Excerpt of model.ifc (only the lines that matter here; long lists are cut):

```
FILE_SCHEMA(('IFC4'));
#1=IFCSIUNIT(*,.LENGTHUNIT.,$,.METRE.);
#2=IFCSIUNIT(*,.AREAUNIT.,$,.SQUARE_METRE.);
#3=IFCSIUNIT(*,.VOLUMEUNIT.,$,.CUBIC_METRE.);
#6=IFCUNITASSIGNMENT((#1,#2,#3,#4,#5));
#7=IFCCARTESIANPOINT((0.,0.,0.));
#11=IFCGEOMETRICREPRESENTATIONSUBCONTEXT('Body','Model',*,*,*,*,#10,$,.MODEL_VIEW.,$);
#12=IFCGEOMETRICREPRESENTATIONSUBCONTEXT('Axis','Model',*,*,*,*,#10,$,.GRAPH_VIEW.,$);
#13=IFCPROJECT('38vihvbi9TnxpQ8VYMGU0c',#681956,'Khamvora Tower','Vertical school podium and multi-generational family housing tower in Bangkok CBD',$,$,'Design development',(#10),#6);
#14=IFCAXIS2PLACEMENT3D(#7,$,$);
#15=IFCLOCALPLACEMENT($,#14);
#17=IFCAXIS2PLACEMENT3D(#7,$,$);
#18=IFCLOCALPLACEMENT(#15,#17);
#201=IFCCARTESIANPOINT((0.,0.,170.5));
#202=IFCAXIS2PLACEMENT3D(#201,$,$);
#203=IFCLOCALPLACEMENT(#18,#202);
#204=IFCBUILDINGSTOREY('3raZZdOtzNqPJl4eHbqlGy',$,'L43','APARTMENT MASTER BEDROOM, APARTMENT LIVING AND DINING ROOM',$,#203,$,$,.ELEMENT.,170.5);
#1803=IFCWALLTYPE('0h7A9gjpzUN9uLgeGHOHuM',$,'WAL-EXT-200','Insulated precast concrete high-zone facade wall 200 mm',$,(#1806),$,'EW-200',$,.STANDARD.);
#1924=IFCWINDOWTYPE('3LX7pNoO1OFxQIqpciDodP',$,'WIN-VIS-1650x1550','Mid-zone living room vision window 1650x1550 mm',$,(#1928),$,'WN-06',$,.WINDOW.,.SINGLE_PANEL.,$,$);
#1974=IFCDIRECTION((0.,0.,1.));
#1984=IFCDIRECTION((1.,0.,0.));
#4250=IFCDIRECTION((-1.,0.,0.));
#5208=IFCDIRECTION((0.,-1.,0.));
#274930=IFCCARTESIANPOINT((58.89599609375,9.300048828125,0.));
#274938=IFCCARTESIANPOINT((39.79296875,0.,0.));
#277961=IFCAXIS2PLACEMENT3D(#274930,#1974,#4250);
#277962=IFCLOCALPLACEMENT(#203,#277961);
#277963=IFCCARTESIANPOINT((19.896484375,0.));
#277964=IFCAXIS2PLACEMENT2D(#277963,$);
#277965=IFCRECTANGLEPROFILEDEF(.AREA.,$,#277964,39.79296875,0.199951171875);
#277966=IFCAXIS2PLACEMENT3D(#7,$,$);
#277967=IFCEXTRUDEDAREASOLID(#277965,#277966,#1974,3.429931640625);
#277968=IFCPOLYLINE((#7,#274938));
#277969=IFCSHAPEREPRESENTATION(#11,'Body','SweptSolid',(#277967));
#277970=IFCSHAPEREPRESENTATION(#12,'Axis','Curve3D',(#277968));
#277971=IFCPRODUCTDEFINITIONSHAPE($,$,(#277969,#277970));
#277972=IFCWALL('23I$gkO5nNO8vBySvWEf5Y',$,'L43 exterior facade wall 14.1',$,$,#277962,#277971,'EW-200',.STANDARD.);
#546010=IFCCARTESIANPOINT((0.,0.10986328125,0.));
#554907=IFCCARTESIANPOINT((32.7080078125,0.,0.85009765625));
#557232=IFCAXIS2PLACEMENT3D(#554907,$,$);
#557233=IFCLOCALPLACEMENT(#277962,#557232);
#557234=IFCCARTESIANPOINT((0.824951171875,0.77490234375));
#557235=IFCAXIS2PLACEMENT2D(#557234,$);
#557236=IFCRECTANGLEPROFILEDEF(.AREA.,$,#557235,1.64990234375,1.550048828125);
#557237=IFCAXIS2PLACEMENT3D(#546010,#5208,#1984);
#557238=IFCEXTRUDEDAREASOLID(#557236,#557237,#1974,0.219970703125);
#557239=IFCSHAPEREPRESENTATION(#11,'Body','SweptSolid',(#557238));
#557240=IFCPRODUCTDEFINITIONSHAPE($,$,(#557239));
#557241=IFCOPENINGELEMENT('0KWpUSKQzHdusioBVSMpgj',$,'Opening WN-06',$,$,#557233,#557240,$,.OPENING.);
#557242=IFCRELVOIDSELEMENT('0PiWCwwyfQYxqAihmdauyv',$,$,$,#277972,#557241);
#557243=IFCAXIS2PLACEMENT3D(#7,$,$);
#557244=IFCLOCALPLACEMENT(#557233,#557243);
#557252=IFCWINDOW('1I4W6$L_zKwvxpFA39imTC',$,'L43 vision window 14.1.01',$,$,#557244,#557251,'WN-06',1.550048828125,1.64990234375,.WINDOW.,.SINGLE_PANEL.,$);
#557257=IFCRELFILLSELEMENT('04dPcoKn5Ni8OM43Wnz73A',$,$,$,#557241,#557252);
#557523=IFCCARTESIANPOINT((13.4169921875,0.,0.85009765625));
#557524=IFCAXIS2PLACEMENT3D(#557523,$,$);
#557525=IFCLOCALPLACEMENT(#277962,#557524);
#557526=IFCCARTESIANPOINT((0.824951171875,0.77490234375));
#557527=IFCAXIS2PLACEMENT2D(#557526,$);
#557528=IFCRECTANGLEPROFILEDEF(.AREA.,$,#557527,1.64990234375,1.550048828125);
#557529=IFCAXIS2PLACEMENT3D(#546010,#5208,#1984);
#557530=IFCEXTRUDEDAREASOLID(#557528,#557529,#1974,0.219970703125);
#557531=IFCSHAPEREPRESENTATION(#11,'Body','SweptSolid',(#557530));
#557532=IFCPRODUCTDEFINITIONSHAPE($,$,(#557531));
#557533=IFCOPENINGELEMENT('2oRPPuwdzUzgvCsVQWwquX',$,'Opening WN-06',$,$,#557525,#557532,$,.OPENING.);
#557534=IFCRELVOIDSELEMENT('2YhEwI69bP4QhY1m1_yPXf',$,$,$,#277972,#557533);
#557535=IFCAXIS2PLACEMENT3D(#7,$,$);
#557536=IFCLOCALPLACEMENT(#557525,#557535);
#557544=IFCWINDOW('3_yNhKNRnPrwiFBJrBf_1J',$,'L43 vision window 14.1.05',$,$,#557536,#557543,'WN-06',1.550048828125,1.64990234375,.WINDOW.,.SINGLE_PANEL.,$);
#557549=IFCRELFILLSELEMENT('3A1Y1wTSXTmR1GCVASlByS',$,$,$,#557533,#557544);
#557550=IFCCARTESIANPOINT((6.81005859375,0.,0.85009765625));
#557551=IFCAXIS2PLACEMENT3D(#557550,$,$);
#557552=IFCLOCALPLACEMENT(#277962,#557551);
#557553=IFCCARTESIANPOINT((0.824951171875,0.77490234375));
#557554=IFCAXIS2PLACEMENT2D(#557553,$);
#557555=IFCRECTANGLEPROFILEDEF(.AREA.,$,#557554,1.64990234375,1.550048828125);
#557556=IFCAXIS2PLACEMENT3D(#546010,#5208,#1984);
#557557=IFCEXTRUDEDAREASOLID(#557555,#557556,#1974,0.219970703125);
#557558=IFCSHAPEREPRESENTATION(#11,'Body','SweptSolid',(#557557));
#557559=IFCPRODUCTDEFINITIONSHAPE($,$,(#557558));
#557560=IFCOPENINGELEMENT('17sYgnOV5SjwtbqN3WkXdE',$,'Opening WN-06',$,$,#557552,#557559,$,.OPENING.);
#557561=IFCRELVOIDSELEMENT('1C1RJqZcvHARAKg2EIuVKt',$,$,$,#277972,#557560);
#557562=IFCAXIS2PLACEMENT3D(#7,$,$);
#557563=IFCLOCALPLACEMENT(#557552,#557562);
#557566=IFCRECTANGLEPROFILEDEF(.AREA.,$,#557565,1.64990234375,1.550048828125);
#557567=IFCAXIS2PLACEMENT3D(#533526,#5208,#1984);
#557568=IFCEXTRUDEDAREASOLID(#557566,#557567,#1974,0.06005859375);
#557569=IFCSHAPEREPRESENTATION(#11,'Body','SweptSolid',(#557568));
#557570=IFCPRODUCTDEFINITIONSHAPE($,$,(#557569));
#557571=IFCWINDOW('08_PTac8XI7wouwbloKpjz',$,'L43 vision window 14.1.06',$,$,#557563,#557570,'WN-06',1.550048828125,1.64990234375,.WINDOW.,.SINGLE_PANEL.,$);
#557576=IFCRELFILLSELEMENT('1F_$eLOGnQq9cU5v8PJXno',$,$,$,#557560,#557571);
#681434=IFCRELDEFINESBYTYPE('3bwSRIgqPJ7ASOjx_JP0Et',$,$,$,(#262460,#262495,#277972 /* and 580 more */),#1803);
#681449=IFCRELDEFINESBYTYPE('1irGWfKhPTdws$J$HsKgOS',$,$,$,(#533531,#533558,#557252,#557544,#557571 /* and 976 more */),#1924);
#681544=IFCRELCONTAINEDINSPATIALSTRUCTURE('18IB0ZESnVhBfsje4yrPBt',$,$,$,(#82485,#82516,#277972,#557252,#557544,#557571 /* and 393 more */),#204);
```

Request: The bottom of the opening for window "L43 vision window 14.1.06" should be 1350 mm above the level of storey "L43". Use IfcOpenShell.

```python
import numpy as np
import ifcopenshell
import ifcopenshell.api.geometry
import ifcopenshell.geom
import ifcopenshell.util.element
import ifcopenshell.util.placement
import ifcopenshell.util.shape
import ifcopenshell.util.unit

model = ifcopenshell.open("model.ifc")
unit_scale = ifcopenshell.util.unit.calculate_unit_scale(model)

window = model.by_guid("08_PTac8XI7wouwbloKpjz")
opening = window.FillsVoids[0].RelatingOpeningElement
storey = ifcopenshell.util.element.get_container(window, ifc_class="IfcBuildingStorey")
level = ifcopenshell.util.placement.get_local_placement(storey.ObjectPlacement)[2, 3]

# The opening's origin need not be at the sill, so measure its lowest point.
shape = ifcopenshell.geom.create_shape(ifcopenshell.geom.settings(), opening)
bottom = ifcopenshell.util.shape.get_shape_bottom_elevation(shape, shape.geometry) / unit_scale
dz = level + 1.35 - bottom

shift = np.array([0.0, 0.0, dz])
# The window is placed relative to its opening, so it follows when the opening moves.
matrix = ifcopenshell.util.placement.get_local_placement(opening.ObjectPlacement)
matrix[:3, 3] += shift
ifcopenshell.api.geometry.edit_object_placement(
    model, product=opening, matrix=matrix, is_si=False, should_transform_children=True
)

print(f"moved by {dz * unit_scale:+.3f} m")

model.write("model-out.ifc")
```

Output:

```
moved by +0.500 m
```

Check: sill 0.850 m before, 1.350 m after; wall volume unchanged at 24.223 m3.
